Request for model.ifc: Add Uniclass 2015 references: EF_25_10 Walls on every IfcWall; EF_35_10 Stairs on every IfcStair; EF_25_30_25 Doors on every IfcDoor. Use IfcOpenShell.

First a look at what the model holds.

```python
import ifcopenshell

model = ifcopenshell.open("model.ifc")
print(model.schema)
print("classifications:", [c.Name for c in model.by_type("IfcClassification")])
for ifc_class in ("IfcDoor", "IfcRoof", "IfcStair", "IfcWall", "IfcWindow"):
    print(ifc_class, len(model.by_type(ifc_class)))
```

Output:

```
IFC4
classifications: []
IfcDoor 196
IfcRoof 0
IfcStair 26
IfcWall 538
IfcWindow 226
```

```python
import ifcopenshell
import ifcopenshell.api.classification

model = ifcopenshell.open("model.ifc")

system = ifcopenshell.api.classification.add_classification(model, classification="Uniclass 2015")

codes = {
    "IfcWall": ("EF_25_10", "Walls"),
    "IfcStair": ("EF_35_10", "Stairs"),
    "IfcDoor": ("EF_25_30_25", "Doors"),
}
for ifc_class, (code, name) in codes.items():
    products = model.by_type(ifc_class)
    ifcopenshell.api.classification.add_reference(
        model, products=products, classification=system, identification=code, name=name
    )
    print(code, len(products))

model.write("model_updated.ifc")
```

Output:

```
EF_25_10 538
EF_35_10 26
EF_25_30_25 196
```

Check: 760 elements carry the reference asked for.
